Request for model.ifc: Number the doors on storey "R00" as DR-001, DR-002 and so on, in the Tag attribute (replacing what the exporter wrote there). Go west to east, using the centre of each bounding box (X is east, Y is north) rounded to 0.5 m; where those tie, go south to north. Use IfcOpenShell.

First a look at what the model holds.

```python
import ifcopenshell
import ifcopenshell.util.element
import ifcopenshell.util.placement

model = ifcopenshell.open("model.ifc")
print(model.schema)
storey = next(s for s in model.by_type("IfcBuildingStorey") if s.Name == "R00")
doors = [e for e in ifcopenshell.util.element.get_decomposition(storey) if e.is_a("IfcDoor")]
for e in sorted(doors, key=lambda e: e.id()):
    origin = ifcopenshell.util.placement.get_local_placement(e.ObjectPlacement)[:3, 3]
    print(e.id(), e.Tag, e.Name, origin.round(2) + 0.0, sep=" | ")
```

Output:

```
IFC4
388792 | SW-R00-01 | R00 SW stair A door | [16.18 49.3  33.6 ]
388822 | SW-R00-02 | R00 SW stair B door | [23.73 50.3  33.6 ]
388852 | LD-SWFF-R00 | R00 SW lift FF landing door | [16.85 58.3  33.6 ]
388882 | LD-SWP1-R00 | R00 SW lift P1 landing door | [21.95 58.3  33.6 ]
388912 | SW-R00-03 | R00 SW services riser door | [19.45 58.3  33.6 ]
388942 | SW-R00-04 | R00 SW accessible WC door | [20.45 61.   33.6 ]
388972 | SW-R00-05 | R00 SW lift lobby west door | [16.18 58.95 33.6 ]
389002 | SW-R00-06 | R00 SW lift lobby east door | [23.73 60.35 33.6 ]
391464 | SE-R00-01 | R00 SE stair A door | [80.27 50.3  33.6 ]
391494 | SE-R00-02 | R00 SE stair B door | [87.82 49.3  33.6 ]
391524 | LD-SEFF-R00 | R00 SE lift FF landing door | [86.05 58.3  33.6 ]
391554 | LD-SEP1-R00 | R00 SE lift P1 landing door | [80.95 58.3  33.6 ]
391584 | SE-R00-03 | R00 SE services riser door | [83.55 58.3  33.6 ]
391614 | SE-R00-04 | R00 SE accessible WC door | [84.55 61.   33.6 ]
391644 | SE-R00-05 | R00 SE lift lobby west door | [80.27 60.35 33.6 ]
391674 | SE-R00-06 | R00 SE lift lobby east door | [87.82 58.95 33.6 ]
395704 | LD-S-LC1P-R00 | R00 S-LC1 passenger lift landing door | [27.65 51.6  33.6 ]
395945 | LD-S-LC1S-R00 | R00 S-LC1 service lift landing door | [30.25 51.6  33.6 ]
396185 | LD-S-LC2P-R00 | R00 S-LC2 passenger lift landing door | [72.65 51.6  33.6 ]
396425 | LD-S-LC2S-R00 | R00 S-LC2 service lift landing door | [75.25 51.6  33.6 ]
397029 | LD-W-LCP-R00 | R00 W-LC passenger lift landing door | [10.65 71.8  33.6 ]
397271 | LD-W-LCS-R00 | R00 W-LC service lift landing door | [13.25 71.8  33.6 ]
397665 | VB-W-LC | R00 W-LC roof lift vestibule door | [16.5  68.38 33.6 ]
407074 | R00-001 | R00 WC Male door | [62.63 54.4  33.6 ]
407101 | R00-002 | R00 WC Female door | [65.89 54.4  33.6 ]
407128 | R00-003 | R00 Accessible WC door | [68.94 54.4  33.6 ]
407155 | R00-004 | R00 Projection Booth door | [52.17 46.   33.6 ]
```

```python
import ifcopenshell
import ifcopenshell.geom
import ifcopenshell.util.element
import ifcopenshell.util.shape

model = ifcopenshell.open("model.ifc")
settings = ifcopenshell.geom.settings()
settings.set("use-world-coords", True)


def centre(element):
    shape = ifcopenshell.geom.create_shape(settings, element)
    return ifcopenshell.util.shape.get_bbox_centroid(shape.geometry)


storey = next(s for s in model.by_type("IfcBuildingStorey") if s.Name == "R00")
doors = [e for e in ifcopenshell.util.element.get_decomposition(storey) if e.is_a("IfcDoor")]

# Insertion points can sit at a corner or the storey origin, so sort by the geometry (in metres).
centres = {e: centre(e) for e in doors}
doors.sort(key=lambda e: (round(centres[e][0] / 0.5), centres[e][1]))

for i, e in enumerate(doors, start=1):
    number = f"DR-0{i:02d}"
    e.Tag = number
    print(e.id(), number)

model.write("model_rev.ifc")
```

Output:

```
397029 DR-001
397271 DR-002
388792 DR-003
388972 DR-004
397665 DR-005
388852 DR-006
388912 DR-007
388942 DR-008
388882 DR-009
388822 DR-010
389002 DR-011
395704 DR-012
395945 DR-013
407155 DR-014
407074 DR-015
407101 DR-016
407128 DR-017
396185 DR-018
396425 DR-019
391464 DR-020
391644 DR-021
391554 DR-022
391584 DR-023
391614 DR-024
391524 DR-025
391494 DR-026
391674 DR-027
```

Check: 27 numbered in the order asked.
